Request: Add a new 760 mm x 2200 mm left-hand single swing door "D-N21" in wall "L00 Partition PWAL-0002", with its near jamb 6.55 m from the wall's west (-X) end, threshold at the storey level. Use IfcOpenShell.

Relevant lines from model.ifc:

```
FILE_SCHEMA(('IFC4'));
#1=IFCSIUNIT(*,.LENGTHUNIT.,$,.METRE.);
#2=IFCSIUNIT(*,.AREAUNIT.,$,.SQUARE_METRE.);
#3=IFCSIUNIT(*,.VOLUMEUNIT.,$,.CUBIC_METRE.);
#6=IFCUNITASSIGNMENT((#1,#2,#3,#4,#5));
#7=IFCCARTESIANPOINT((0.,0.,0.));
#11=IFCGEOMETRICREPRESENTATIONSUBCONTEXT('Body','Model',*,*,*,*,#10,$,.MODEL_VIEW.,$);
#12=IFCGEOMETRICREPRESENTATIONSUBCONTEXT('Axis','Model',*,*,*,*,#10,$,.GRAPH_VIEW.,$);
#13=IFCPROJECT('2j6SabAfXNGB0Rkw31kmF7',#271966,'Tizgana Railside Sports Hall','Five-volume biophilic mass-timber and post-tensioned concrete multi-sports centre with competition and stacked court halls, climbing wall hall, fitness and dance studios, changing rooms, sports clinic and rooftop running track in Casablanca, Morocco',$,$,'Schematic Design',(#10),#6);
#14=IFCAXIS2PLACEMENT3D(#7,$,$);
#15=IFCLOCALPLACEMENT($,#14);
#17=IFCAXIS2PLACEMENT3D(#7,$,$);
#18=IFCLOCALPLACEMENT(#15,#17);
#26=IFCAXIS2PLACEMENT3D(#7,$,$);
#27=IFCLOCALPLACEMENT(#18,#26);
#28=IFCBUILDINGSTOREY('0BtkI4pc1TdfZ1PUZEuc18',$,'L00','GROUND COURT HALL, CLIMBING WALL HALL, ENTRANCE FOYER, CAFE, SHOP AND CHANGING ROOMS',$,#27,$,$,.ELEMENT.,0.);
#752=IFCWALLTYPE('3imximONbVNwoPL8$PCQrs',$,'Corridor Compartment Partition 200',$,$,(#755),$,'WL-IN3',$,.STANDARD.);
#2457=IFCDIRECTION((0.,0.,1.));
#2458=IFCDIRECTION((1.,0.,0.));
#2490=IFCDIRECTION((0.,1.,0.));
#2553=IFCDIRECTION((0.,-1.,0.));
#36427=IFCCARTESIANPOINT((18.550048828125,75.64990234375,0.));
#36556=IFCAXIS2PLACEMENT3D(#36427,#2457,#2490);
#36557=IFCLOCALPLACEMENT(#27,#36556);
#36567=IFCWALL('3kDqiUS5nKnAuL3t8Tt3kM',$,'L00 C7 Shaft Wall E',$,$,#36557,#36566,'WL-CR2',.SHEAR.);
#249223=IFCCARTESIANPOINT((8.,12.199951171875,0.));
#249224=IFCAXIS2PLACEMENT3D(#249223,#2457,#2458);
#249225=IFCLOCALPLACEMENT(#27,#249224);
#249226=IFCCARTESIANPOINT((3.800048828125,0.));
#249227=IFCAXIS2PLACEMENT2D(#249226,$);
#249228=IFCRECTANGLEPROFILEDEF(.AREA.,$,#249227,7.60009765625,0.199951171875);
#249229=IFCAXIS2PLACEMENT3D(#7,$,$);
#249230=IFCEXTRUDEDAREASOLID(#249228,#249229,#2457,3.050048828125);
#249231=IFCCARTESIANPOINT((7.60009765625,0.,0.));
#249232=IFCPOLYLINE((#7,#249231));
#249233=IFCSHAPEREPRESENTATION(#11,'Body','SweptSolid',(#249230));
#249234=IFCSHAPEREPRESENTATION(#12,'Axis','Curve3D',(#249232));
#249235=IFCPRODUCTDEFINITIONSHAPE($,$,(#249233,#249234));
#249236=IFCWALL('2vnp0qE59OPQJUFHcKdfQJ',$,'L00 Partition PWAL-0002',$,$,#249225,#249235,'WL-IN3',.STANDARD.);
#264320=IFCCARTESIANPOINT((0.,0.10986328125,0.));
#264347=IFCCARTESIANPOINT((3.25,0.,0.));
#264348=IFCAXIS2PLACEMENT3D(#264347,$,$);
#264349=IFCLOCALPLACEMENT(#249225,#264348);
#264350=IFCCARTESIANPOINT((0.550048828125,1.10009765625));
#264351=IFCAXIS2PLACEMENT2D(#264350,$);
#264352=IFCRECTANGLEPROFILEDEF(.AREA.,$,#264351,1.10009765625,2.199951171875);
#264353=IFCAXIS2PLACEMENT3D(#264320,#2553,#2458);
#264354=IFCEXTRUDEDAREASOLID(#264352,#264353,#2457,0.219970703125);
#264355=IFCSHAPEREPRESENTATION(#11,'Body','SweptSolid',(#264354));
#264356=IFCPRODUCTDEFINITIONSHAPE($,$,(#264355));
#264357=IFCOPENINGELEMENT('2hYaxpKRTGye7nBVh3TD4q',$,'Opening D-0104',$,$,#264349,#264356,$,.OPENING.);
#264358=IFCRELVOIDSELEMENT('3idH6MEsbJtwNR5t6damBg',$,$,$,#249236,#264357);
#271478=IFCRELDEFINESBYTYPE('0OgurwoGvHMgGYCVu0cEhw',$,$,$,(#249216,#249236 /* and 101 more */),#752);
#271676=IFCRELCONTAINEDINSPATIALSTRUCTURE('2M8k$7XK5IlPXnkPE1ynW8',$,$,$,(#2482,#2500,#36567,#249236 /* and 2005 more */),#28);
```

```python
import numpy as np
import ifcopenshell
import ifcopenshell.api.feature
import ifcopenshell.api.geometry
import ifcopenshell.api.root
import ifcopenshell.api.spatial
import ifcopenshell.geom
import ifcopenshell.util.element
import ifcopenshell.util.placement
import ifcopenshell.util.representation
import ifcopenshell.util.shape
import ifcopenshell.util.unit

model = ifcopenshell.open("model.ifc")
unit_scale = ifcopenshell.util.unit.calculate_unit_scale(model)
settings = ifcopenshell.geom.settings()


def volume(element):
    """Net volume in cubic metres, openings subtracted."""
    shape = ifcopenshell.geom.create_shape(settings, element)
    return ifcopenshell.util.shape.get_volume(shape.geometry)


wall = model.by_guid("2vnp0qE59OPQJUFHcKdfQJ")
storey = ifcopenshell.util.element.get_container(wall, ifc_class="IfcBuildingStorey")
context = ifcopenshell.util.representation.get_context(model, "Model", "Body", "MODEL_VIEW")
before = volume(wall)

width, height, from_end, sill = 0.76, 2.2, 6.55, 0.0  # metres

# The wall runs along its own X axis, and the end named is its -X end.
wall_shape = ifcopenshell.geom.create_shape(settings, wall)
x, y, z = ifcopenshell.util.shape.get_vertices(wall_shape.geometry).T
start = x.min() + from_end
face, thickness = float(y.min()), float(y.max() - y.min())
wall_matrix = ifcopenshell.util.placement.get_local_placement(wall.ObjectPlacement)
level = ifcopenshell.util.placement.get_local_placement(storey.ObjectPlacement)[2, 3]


def in_wall(x, y):
    """Placement at x, y metres in the wall's axes, at sill height."""
    matrix = wall_matrix.copy()
    matrix[:, 3] = wall_matrix @ np.array([x / unit_scale, y / unit_scale, 0.0, 1.0])
    matrix[2, 3] = level + sill / unit_scale
    return matrix


# Opening: a box that overshoots both wall faces by 50 mm.
opening = ifcopenshell.api.root.create_entity(model, ifc_class="IfcOpeningElement", predefined_type="OPENING")
box = ifcopenshell.api.geometry.add_wall_representation(
    model, context=context, length=width, height=height, thickness=thickness + 0.1
)
ifcopenshell.api.geometry.assign_representation(model, product=opening, representation=box)
ifcopenshell.api.geometry.edit_object_placement(model, product=opening, matrix=in_wall(start, face - 0.05), is_si=False)
ifcopenshell.api.feature.add_feature(model, feature=opening, element=wall)

door = ifcopenshell.api.root.create_entity(model, ifc_class="IfcDoor", name="D-N21", predefined_type="DOOR")
door.OverallWidth, door.OverallHeight = width / unit_scale, height / unit_scale
door.OperationType = "SINGLE_SWING_LEFT"
body = ifcopenshell.api.geometry.add_door_representation(
    model,
    context=context,
    overall_width=door.OverallWidth,
    overall_height=door.OverallHeight,
    operation_type="SINGLE_SWING_LEFT",
    lining_properties={"LiningDepth": thickness / unit_scale, "ThresholdDepth": thickness / unit_scale},
)
ifcopenshell.api.geometry.assign_representation(model, product=door, representation=body)
ifcopenshell.api.spatial.assign_container(model, products=[door], relating_structure=storey)
ifcopenshell.api.feature.add_filling(model, opening=opening, element=door)

# The lining spans the wall, so the door starts at the wall face.
ifcopenshell.api.geometry.edit_object_placement(model, product=door, matrix=in_wall(start, face), is_si=False)

after = volume(wall)

print(f"wall volume {before:.3f} -> {after:.3f} m3")

model.write("model_rev.ifc")
```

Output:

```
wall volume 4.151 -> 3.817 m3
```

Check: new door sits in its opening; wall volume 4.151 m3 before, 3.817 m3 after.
